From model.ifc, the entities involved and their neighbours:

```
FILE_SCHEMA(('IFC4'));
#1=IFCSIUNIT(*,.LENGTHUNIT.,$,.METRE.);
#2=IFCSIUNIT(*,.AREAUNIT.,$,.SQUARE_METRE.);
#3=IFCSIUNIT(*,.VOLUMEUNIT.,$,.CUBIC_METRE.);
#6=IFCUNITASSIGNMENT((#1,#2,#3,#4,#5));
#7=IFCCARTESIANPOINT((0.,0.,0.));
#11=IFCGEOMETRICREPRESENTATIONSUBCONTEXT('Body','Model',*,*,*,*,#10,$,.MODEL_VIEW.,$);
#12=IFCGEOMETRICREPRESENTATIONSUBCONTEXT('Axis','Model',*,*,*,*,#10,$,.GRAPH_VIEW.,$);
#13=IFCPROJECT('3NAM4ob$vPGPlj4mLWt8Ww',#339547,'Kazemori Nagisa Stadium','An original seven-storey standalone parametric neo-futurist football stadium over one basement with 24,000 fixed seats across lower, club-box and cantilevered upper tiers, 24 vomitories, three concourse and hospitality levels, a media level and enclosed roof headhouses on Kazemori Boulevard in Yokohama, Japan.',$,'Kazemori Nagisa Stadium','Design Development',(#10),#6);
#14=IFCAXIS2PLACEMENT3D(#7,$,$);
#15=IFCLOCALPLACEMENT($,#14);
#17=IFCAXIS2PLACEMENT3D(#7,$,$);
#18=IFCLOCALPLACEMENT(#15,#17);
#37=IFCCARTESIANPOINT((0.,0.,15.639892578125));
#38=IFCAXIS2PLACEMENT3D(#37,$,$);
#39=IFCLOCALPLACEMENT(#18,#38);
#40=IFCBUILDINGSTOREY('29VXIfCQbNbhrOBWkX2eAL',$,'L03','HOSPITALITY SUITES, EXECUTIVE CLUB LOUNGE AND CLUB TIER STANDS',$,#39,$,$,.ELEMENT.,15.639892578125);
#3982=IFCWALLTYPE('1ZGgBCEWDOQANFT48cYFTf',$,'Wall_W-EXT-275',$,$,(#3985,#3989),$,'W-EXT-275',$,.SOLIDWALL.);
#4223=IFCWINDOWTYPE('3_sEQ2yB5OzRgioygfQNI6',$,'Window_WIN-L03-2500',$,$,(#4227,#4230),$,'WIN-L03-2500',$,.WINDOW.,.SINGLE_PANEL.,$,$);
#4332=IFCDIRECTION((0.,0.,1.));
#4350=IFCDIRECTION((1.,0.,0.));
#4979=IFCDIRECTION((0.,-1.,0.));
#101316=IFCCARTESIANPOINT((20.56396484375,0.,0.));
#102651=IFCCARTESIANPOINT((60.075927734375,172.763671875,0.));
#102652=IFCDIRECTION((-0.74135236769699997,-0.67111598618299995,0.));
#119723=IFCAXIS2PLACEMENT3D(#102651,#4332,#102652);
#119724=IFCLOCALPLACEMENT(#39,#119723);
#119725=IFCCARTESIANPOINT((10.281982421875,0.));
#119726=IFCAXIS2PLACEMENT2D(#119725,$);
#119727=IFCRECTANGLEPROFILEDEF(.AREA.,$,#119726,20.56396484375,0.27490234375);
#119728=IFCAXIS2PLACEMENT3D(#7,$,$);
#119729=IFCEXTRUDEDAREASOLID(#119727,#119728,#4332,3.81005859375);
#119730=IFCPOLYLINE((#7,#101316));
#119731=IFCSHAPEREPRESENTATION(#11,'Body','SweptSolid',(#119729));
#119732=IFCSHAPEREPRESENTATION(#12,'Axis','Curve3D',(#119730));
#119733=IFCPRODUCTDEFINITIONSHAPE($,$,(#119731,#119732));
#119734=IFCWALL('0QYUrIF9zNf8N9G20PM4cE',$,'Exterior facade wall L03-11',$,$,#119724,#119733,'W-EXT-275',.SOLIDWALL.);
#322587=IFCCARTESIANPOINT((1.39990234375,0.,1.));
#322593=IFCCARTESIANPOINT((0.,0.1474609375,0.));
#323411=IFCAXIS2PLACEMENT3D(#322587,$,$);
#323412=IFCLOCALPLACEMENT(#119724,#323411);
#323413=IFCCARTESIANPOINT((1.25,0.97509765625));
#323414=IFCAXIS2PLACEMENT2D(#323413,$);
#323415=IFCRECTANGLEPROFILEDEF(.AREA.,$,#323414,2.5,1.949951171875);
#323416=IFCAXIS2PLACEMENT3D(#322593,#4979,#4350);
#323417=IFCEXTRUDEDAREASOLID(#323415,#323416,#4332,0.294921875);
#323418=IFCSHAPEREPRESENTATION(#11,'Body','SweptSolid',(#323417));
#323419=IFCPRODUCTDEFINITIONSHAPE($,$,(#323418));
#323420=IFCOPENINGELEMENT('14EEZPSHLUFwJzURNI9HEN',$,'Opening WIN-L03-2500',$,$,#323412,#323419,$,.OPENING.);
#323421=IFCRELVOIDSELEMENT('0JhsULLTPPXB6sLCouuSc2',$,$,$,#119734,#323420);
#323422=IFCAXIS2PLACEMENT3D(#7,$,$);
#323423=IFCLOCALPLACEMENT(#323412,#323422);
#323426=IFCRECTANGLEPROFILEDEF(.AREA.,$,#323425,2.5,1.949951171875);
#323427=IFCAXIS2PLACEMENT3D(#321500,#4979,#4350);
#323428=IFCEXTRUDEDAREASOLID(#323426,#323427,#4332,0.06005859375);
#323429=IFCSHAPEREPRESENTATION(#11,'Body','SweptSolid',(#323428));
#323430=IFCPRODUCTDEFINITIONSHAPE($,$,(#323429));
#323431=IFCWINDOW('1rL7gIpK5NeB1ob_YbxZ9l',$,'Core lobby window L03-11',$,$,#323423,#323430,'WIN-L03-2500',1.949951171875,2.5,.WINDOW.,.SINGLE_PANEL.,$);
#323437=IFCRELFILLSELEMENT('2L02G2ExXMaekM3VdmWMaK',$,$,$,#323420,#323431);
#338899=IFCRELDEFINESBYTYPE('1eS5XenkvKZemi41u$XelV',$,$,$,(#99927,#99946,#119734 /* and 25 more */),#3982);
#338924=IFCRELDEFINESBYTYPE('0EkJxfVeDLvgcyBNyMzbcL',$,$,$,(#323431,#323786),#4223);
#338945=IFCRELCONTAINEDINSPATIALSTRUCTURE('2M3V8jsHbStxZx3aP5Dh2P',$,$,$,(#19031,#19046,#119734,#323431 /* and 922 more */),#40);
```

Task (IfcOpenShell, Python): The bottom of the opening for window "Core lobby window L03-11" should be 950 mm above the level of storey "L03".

```python
import numpy as np
import ifcopenshell
import ifcopenshell.api.geometry
import ifcopenshell.geom
import ifcopenshell.util.element
import ifcopenshell.util.placement
import ifcopenshell.util.shape
import ifcopenshell.util.unit

model = ifcopenshell.open("model.ifc")
unit_scale = ifcopenshell.util.unit.calculate_unit_scale(model)

window = model.by_id(323431)
opening = window.FillsVoids[0].RelatingOpeningElement
storey = ifcopenshell.util.element.get_container(window, ifc_class="IfcBuildingStorey")
level = ifcopenshell.util.placement.get_local_placement(storey.ObjectPlacement)[2, 3]

# The opening's origin need not be at the sill, so measure its lowest point.
shape = ifcopenshell.geom.create_shape(ifcopenshell.geom.settings(), opening)
bottom = ifcopenshell.util.shape.get_shape_bottom_elevation(shape, shape.geometry) / unit_scale
dz = level + 0.95 / unit_scale - bottom

shift = np.array([0.0, 0.0, dz])
# The window is placed relative to its opening, so it follows when the opening moves.
matrix = ifcopenshell.util.placement.get_local_placement(opening.ObjectPlacement)
matrix[:3, 3] += shift
ifcopenshell.api.geometry.edit_object_placement(
    model, product=opening, matrix=matrix, is_si=False, should_transform_children=True
)

print(f"moved by {dz * unit_scale:+.3f} m")

model.write("model_rev.ifc")
```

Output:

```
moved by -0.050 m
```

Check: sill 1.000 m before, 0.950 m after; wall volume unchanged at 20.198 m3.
